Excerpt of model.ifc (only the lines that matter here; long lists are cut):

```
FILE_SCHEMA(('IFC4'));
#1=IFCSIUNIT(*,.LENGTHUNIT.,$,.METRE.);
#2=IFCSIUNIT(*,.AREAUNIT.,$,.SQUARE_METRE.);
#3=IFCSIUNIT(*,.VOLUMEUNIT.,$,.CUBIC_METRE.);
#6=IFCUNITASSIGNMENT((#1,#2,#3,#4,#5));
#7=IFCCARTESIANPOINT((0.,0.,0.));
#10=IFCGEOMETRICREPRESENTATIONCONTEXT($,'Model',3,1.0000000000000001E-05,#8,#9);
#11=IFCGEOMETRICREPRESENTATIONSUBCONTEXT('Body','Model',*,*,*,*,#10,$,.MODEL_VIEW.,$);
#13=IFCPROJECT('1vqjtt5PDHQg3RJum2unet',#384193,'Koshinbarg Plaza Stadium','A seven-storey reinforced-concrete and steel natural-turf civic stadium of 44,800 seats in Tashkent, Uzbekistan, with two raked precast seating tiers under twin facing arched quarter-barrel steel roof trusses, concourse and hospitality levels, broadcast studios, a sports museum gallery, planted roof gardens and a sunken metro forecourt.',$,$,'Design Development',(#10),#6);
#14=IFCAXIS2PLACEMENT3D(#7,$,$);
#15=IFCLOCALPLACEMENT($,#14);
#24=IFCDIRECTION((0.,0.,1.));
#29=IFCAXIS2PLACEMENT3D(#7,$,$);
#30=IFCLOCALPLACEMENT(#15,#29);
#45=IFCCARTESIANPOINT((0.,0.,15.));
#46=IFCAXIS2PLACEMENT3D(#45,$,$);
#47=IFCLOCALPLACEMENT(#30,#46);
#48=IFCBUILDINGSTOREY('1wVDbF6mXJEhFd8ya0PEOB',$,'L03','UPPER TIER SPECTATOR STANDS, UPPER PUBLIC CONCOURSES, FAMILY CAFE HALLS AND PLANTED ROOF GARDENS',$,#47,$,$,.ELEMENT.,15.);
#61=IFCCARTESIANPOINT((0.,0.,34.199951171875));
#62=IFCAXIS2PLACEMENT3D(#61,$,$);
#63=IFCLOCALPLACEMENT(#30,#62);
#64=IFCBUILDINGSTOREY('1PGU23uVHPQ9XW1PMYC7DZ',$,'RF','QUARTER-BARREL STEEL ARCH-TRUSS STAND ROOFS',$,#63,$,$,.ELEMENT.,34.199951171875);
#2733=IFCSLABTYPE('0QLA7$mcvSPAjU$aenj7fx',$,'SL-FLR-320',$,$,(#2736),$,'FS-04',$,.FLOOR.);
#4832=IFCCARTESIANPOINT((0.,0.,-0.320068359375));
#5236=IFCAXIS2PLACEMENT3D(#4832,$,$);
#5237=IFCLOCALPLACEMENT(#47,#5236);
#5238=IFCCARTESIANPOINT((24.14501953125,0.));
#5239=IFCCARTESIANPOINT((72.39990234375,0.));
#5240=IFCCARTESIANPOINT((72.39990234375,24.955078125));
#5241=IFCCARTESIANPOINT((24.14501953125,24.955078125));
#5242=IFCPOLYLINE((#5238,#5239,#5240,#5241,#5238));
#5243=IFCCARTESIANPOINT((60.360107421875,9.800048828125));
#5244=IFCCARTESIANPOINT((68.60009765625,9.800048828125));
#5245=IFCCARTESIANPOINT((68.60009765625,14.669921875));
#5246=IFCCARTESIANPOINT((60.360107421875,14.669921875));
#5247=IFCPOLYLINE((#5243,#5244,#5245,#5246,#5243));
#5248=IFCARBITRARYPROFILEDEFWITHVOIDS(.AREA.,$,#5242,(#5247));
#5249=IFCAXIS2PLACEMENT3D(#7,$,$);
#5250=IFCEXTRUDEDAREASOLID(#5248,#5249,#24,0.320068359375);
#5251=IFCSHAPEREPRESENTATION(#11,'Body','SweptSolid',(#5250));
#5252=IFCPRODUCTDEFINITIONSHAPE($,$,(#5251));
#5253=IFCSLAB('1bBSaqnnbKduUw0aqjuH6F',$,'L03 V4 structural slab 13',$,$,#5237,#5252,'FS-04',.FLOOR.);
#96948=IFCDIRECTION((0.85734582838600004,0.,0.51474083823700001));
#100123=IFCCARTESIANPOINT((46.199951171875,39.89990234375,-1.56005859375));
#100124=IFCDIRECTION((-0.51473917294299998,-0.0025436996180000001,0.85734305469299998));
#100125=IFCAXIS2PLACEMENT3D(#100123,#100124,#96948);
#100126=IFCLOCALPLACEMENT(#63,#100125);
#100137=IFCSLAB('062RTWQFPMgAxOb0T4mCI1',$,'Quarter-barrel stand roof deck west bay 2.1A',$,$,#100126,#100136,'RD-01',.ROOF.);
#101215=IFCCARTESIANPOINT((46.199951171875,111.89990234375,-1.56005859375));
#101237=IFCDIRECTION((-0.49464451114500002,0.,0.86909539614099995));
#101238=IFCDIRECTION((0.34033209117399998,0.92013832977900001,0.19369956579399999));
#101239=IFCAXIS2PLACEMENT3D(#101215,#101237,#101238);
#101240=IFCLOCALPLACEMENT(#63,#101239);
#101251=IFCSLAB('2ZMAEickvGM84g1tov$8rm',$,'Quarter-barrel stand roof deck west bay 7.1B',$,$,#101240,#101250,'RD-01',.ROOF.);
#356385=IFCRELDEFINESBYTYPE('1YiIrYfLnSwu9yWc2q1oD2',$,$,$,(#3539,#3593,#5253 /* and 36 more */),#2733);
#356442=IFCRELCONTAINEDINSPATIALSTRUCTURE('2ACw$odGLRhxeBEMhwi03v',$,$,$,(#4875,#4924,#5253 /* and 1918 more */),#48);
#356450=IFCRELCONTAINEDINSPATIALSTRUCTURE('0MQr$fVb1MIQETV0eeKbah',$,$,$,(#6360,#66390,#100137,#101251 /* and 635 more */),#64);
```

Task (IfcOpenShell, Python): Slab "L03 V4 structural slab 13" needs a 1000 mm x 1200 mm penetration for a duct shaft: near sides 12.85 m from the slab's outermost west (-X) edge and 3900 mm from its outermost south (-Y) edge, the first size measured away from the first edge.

```python
import numpy as np
import ifcopenshell
import ifcopenshell.api.feature
import ifcopenshell.api.geometry
import ifcopenshell.api.root
import ifcopenshell.geom
import ifcopenshell.util.placement
import ifcopenshell.util.representation
import ifcopenshell.util.shape
import ifcopenshell.util.unit

model = ifcopenshell.open("model.ifc")
unit_scale = ifcopenshell.util.unit.calculate_unit_scale(model)
settings = ifcopenshell.geom.settings()


def volume(element):
    """Net volume in cubic metres, openings subtracted."""
    shape = ifcopenshell.geom.create_shape(settings, element)
    return ifcopenshell.util.shape.get_volume(shape.geometry)


slab = model.by_guid("1bBSaqnnbKduUw0aqjuH6F")
before = volume(slab)

# Extent in the slab's own axes, in metres. The edges named are its -X and -Y sides.
slab_shape = ifcopenshell.geom.create_shape(settings, slab)
vertices = ifcopenshell.util.shape.get_vertices(slab_shape.geometry)
x_min, y_min, bottom = vertices.min(axis=0)
top = vertices[:, 2].max()

opening = ifcopenshell.api.root.create_entity(model, ifc_class="IfcOpeningElement", name="Duct shaft opening", predefined_type="OPENING")
context = ifcopenshell.util.representation.get_context(model, "Model", "Body", "MODEL_VIEW")
width, depth = 1, 1.2
outline = [(0.0, 0.0), (width, 0.0), (width, depth), (0.0, depth), (0.0, 0.0)]
# Overshoot both faces by 50 mm so the cut is clean.
shape = ifcopenshell.api.geometry.add_slab_representation(
    model, context=context, depth=top - bottom + 0.1, polyline=outline
)
ifcopenshell.api.geometry.assign_representation(model, product=opening, representation=shape)

matrix = ifcopenshell.util.placement.get_local_placement(slab.ObjectPlacement)
matrix[:, 3] = matrix @ np.append(np.array([x_min + 12.85, y_min + 3.9, bottom - 0.05]) / unit_scale, 1.0)
ifcopenshell.api.geometry.edit_object_placement(model, product=opening, matrix=matrix, is_si=False)
ifcopenshell.api.feature.add_feature(model, feature=opening, element=slab)

after = volume(slab)

print(f"slab volume {before:.3f} -> {after:.3f} m3")

model.write("model_updated.ifc")
```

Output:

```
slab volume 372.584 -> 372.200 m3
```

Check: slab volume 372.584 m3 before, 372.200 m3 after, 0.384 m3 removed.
